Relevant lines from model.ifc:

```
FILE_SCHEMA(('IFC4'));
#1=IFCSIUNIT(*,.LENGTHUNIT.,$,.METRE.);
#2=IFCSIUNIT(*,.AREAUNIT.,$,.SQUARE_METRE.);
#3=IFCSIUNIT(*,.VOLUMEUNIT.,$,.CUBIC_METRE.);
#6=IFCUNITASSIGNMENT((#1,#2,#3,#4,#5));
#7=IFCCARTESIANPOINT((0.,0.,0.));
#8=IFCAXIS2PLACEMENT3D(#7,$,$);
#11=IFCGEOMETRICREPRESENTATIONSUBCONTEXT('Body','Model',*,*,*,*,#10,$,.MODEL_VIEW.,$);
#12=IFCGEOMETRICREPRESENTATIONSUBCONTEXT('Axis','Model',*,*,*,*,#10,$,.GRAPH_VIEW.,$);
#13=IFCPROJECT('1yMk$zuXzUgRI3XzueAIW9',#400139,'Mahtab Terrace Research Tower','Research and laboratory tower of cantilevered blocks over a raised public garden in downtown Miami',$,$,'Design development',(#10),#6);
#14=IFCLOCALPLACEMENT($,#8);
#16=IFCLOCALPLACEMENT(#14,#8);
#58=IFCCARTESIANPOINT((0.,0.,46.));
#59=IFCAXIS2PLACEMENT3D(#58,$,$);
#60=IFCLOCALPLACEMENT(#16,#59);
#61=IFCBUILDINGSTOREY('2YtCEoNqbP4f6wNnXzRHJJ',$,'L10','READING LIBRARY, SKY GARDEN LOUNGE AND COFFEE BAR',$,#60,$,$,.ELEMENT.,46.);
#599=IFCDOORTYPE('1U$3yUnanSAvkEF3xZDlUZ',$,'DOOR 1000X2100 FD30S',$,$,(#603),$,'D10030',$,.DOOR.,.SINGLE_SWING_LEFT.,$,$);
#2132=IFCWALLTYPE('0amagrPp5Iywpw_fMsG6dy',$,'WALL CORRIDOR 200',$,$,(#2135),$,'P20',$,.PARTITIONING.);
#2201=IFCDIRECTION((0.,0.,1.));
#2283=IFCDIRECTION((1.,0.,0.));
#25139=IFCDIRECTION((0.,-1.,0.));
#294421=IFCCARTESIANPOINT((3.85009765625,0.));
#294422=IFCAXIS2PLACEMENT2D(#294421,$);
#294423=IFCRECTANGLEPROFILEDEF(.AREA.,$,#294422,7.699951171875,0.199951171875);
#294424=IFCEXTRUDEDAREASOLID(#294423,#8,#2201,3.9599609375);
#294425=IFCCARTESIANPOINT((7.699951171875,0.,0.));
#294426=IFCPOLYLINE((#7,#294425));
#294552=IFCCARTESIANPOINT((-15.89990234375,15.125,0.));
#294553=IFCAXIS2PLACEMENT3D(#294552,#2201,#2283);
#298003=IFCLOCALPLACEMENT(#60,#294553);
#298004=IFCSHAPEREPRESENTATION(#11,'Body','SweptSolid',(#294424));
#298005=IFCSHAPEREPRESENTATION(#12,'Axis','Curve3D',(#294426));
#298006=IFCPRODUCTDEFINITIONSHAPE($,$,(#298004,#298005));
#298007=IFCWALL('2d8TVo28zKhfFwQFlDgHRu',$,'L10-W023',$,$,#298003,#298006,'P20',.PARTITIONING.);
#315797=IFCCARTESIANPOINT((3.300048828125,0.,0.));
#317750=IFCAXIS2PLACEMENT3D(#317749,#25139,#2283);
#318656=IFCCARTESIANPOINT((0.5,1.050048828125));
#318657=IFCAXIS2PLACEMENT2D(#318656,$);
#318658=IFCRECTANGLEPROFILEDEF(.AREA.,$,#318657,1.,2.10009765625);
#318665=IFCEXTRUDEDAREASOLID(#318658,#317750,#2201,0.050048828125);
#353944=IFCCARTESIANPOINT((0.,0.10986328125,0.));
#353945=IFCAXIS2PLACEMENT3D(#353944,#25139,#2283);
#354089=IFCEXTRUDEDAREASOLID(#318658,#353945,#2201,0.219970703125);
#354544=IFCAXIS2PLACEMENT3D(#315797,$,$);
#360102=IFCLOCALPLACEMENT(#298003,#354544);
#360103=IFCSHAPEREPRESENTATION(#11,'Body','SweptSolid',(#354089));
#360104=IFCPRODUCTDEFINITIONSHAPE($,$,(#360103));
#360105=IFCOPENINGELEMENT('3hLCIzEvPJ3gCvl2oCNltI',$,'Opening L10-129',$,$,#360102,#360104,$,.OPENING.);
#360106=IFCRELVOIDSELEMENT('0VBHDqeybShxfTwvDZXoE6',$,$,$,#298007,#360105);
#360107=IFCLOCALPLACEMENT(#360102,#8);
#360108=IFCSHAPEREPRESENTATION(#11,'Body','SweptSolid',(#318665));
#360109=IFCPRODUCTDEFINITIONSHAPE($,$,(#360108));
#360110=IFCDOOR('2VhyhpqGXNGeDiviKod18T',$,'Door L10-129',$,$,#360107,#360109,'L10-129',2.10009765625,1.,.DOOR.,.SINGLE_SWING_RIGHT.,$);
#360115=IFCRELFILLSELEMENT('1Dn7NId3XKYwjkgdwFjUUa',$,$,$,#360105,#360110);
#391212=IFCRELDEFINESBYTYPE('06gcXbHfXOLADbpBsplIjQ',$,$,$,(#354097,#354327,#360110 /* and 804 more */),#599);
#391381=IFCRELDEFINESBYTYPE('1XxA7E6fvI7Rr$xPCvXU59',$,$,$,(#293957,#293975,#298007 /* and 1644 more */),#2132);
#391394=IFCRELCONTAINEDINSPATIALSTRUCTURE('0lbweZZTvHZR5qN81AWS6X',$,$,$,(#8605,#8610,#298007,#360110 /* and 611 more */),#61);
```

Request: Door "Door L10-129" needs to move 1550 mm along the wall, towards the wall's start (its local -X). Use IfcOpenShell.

```python
import ifcopenshell
import ifcopenshell.api.geometry
import ifcopenshell.util.placement

model = ifcopenshell.open("model.ifc")

door = model.by_guid("2VhyhpqGXNGeDiviKod18T")
opening = door.FillsVoids[0].RelatingOpeningElement
wall = opening.VoidsElements[0].RelatingBuildingElement

wall_matrix = ifcopenshell.util.placement.get_local_placement(wall.ObjectPlacement)
shift = wall_matrix[:3, 0] * -1.55
before = ifcopenshell.util.placement.get_local_placement(door.ObjectPlacement)[:3, 3].copy()

# The door is placed relative to its opening, so it follows when the opening moves.
matrix = ifcopenshell.util.placement.get_local_placement(opening.ObjectPlacement)
matrix[:3, 3] += shift
ifcopenshell.api.geometry.edit_object_placement(
    model, product=opening, matrix=matrix, is_si=False, should_transform_children=True
)

after = ifcopenshell.util.placement.get_local_placement(door.ObjectPlacement)[:3, 3]
print("door moved by", (after - before).round(3) + 0.0)

model.write("model_rev.ifc")
```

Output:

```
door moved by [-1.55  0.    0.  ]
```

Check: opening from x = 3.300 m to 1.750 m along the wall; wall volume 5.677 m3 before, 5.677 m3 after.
